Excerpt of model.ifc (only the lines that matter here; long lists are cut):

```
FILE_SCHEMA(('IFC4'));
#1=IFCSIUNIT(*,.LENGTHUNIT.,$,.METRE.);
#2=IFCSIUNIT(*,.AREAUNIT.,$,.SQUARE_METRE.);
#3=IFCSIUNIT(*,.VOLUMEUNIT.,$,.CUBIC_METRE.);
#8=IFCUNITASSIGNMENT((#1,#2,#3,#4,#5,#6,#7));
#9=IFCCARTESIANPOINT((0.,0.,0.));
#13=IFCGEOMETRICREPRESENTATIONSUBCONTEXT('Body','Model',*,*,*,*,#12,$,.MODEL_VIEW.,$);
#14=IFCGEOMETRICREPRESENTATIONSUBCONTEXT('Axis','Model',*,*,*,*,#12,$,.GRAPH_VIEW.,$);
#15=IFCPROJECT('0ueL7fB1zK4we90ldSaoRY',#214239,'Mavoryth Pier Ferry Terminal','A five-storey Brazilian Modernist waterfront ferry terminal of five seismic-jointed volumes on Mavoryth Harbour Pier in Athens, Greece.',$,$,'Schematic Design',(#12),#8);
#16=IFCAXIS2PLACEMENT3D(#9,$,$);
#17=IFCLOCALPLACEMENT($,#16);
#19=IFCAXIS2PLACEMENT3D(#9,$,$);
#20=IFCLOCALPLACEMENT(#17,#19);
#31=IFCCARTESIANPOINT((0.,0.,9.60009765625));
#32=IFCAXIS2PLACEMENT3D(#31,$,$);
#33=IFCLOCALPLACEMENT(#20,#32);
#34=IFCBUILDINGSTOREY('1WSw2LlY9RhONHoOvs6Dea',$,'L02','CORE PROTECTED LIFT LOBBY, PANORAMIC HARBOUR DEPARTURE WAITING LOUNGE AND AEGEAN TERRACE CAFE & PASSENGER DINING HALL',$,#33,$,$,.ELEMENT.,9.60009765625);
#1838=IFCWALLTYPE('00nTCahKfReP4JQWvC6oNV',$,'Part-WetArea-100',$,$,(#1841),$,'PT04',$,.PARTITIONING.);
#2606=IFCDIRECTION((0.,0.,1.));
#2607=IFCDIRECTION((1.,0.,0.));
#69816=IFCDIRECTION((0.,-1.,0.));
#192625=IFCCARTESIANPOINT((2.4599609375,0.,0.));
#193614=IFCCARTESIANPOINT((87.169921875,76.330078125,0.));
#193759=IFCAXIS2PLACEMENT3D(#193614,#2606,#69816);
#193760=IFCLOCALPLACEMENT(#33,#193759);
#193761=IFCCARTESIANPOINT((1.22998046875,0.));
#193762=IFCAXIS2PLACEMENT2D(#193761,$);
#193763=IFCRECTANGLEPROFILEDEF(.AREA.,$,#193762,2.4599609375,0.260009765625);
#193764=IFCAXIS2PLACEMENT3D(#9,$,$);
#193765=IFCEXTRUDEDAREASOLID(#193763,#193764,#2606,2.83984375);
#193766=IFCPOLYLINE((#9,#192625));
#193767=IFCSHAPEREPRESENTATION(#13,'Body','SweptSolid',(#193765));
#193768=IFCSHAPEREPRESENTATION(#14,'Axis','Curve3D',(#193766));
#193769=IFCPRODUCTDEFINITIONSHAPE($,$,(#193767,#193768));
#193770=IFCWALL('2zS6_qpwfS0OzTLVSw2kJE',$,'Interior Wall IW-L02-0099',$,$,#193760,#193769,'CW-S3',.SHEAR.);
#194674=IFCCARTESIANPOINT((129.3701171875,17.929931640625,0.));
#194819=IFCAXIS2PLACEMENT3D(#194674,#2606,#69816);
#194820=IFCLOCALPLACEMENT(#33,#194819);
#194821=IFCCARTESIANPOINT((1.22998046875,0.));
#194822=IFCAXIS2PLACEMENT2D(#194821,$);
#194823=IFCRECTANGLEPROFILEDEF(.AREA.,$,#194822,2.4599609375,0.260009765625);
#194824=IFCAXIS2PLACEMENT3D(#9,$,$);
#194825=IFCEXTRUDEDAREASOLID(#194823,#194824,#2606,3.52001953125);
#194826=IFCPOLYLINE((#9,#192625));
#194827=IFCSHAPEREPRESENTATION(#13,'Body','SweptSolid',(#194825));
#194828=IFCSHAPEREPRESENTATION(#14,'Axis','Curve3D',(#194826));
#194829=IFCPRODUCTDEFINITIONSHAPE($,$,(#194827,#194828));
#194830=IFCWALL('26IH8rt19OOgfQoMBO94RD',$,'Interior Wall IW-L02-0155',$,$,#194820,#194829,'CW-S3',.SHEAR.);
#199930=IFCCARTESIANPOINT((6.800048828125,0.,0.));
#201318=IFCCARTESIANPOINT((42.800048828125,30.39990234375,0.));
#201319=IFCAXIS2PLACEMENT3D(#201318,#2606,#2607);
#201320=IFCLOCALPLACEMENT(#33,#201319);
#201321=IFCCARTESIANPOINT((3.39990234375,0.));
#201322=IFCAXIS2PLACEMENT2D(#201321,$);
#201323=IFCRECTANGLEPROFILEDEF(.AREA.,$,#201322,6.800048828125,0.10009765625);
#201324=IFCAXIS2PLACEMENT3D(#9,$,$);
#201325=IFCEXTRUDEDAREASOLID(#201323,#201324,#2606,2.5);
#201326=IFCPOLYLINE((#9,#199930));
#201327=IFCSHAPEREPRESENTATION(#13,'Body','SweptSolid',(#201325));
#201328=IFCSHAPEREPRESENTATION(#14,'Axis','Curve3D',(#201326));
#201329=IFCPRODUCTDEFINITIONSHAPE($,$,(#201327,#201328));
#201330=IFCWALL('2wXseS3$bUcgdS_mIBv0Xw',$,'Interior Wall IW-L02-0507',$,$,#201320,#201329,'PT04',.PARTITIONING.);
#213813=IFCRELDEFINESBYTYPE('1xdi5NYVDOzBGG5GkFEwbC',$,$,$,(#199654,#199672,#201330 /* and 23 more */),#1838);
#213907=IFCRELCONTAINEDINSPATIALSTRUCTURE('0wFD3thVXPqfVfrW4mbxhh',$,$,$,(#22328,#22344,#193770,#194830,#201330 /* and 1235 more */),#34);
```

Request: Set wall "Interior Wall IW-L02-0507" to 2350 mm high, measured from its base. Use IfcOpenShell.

```python
import ifcopenshell
import ifcopenshell.geom
import ifcopenshell.util.representation
import ifcopenshell.util.shape
import ifcopenshell.util.unit

model = ifcopenshell.open("model.ifc")
unit_scale = ifcopenshell.util.unit.calculate_unit_scale(model)
settings = ifcopenshell.geom.settings()


def volume(element):
    """Net volume in cubic metres, openings subtracted."""
    shape = ifcopenshell.geom.create_shape(settings, element)
    return ifcopenshell.util.shape.get_volume(shape.geometry)


wall = model.by_id(201330)
before = volume(wall)

body = ifcopenshell.util.representation.get_representation(wall, "Model", "Body")
solid = body.Items[0]
old_height = solid.Depth
solid.Depth = 2.35 / unit_scale
after = volume(wall)

print(f"height {old_height:g} -> {solid.Depth:g}, volume {before:.3f} -> {after:.3f} m3")

model.write("model_updated.ifc")
```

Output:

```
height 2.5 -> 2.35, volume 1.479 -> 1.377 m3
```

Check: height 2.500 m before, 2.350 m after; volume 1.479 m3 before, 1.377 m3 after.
